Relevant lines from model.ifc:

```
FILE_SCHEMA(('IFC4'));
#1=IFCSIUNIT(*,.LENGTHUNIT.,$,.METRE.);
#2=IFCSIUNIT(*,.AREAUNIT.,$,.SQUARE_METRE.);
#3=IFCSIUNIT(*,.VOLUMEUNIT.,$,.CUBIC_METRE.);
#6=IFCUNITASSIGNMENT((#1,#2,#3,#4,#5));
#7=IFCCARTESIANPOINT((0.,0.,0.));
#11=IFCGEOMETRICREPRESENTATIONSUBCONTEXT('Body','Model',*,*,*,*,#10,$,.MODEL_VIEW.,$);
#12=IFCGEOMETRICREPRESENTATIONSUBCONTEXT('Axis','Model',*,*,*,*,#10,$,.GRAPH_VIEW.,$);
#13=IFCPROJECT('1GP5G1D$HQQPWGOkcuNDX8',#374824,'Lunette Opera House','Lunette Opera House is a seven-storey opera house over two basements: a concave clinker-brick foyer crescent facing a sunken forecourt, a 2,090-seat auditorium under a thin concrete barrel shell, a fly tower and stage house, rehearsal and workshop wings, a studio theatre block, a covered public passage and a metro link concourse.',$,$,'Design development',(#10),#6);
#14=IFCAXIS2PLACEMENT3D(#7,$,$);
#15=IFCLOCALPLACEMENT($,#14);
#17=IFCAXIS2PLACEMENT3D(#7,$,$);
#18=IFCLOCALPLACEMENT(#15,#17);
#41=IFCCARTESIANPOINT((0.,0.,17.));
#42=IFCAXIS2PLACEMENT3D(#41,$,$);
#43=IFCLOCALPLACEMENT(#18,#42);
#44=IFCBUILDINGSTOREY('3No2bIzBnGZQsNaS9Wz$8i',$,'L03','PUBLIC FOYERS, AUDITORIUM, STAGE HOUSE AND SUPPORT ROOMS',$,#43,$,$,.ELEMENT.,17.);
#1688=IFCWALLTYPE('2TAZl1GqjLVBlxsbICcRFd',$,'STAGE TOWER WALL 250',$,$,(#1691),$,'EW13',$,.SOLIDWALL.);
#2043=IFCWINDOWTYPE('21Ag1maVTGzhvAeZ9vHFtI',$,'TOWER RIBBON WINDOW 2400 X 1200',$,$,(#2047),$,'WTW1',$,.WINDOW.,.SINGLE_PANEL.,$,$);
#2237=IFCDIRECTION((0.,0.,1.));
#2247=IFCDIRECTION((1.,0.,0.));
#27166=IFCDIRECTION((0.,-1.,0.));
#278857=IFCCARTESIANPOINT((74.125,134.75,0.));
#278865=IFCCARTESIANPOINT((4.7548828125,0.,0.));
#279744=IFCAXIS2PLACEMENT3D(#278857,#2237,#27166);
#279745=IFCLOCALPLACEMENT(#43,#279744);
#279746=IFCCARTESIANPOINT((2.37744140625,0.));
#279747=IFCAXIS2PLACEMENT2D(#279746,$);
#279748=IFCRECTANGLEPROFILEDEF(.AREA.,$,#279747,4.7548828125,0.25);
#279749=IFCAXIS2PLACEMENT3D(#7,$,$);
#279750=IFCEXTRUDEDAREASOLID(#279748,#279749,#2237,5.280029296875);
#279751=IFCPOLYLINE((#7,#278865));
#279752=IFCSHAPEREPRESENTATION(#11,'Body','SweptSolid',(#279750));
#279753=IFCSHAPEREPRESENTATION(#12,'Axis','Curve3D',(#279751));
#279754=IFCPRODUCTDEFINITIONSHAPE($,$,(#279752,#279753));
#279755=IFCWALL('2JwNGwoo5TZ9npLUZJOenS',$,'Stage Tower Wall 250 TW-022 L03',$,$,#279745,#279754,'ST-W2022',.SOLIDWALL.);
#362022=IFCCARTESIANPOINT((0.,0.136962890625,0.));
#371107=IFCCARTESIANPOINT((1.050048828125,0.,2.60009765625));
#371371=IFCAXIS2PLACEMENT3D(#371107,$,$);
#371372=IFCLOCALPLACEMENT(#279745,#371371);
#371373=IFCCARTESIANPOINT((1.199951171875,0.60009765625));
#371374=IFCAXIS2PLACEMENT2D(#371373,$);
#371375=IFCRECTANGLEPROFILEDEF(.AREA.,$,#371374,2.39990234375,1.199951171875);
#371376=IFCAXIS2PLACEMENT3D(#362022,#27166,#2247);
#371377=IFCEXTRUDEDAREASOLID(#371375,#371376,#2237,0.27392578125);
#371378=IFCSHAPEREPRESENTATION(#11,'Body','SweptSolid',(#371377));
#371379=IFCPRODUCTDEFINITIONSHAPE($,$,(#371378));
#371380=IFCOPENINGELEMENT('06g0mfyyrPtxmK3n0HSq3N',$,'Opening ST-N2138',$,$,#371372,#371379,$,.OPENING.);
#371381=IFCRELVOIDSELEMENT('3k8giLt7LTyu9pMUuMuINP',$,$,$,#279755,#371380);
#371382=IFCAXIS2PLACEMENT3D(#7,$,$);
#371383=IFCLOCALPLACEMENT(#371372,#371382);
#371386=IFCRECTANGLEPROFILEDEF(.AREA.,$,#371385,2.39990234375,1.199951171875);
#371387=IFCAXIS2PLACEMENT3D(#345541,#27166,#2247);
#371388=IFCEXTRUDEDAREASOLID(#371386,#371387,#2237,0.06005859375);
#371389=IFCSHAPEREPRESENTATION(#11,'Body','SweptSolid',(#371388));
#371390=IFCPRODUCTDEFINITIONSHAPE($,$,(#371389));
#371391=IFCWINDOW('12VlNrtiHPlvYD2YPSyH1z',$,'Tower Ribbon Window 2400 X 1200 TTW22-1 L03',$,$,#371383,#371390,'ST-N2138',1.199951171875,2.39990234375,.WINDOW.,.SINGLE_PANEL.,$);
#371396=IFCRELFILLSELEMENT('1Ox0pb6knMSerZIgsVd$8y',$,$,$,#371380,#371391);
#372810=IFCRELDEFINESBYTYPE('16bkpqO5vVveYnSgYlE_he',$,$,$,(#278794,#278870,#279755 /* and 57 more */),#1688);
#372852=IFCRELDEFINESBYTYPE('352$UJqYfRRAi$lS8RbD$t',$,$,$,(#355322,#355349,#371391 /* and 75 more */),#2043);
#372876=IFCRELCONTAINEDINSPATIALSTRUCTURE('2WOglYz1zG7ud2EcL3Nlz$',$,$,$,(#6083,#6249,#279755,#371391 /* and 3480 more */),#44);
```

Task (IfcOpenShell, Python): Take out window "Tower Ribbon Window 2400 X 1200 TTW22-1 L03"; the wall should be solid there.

```python
import ifcopenshell
import ifcopenshell.api.feature
import ifcopenshell.api.root
import ifcopenshell.geom
import ifcopenshell.util.shape

model = ifcopenshell.open("model.ifc")
settings = ifcopenshell.geom.settings()


def volume(element):
    """Net volume in cubic metres, openings subtracted."""
    shape = ifcopenshell.geom.create_shape(settings, element)
    return ifcopenshell.util.shape.get_volume(shape.geometry)


window = model.by_guid("12VlNrtiHPlvYD2YPSyH1z")
opening = window.FillsVoids[0].RelatingOpeningElement
wall = opening.VoidsElements[0].RelatingBuildingElement
before = volume(wall)

ifcopenshell.api.root.remove_product(model, product=window)
ifcopenshell.api.feature.remove_feature(model, feature=opening)

after = volume(wall)

print(f"wall volume {before:.3f} -> {after:.3f} m3")

model.write("model_updated.ifc")
```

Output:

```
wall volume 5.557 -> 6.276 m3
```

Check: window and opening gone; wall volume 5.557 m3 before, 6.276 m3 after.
